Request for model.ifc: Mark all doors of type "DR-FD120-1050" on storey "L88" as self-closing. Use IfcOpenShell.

First a look at what the model holds.

```python
import ifcopenshell
import ifcopenshell.util.element

model = ifcopenshell.open("model.ifc")
print(model.schema)
storey = next(s for s in model.by_type("IfcBuildingStorey") if s.Name == "L88")
doors = [e for e in ifcopenshell.util.element.get_decomposition(storey) if e.is_a("IfcDoor")]
seen = {}
for e in doors:
    element_type = ifcopenshell.util.element.get_type(e)
    key = (element_type.Name if element_type != e and element_type else None, ifcopenshell.util.element.get_pset(e, "Pset_DoorCommon", "SelfClosing"))
    seen[key] = seen.get(key, 0) + 1
for (name, value), count in sorted(seen.items(), key=str):
    print(count, "x", name, "|", value)
```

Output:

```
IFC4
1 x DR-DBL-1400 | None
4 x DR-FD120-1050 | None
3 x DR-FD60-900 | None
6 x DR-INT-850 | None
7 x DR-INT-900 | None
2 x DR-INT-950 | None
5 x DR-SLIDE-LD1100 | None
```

```python
import ifcopenshell
import ifcopenshell.api.pset
import ifcopenshell.util.element

model = ifcopenshell.open("model.ifc")

storey = next(s for s in model.by_type("IfcBuildingStorey") if s.Name == "L88")
doors = [e for e in ifcopenshell.util.element.get_decomposition(storey) if e.is_a("IfcDoor")]

count = 0
for e in doors:
    element_type = ifcopenshell.util.element.get_type(e)
    if element_type in (None, e) or element_type.Name != "DR-FD120-1050":
        continue
    # add_pset returns the element's existing set when there is one.
    pset = ifcopenshell.api.pset.add_pset(model, product=e, name="Pset_DoorCommon")
    ifcopenshell.api.pset.edit_pset(model, pset=pset, properties={"SelfClosing": True})
    count += 1

print(count, "doors updated")

model.write("model_v2.ifc")
```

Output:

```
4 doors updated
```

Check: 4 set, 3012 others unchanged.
